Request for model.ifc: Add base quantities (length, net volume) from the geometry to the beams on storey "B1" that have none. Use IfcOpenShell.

First a look at what the model holds.

```python
import ifcopenshell
import ifcopenshell.util.element
import ifcopenshell.util.unit

model = ifcopenshell.open("model.ifc")
print(model.schema)
for unit_type in ("LENGTHUNIT", "AREAUNIT", "VOLUMEUNIT"):
    print(unit_type, ifcopenshell.util.unit.calculate_unit_scale(model, unit_type))
storey = next(s for s in model.by_type("IfcBuildingStorey") if s.Name == "B1")
beams = [e for e in ifcopenshell.util.element.get_decomposition(storey) if e.is_a("IfcBeam")]
for e in sorted(beams, key=lambda e: e.id()):
    print(e.id(), e.is_a(), e.Name, list(ifcopenshell.util.element.get_psets(e, qtos_only=True)), sep=" | ")
```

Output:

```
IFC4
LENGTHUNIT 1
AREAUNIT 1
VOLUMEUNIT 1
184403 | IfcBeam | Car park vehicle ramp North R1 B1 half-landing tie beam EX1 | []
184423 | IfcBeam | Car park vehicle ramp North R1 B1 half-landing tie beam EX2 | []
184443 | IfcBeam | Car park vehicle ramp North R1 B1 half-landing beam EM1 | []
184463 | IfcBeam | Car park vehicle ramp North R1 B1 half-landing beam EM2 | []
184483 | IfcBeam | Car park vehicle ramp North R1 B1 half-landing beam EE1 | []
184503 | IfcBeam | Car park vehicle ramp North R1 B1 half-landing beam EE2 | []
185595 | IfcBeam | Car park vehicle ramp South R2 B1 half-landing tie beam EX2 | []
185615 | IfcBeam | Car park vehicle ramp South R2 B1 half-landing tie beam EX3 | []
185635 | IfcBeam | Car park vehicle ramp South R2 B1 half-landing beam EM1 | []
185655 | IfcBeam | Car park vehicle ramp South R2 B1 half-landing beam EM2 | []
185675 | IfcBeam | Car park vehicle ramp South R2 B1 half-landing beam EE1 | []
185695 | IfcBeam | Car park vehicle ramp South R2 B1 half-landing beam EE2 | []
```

```python
import ifcopenshell
import ifcopenshell.api.pset
import ifcopenshell.geom
import ifcopenshell.util.element
import ifcopenshell.util.shape
import ifcopenshell.util.unit

model = ifcopenshell.open("model.ifc")
unit_scale = ifcopenshell.util.unit.calculate_unit_scale(model)
volume_scale = ifcopenshell.util.unit.calculate_unit_scale(model, "VOLUMEUNIT")
settings = ifcopenshell.geom.settings()

storey = next(s for s in model.by_type("IfcBuildingStorey") if s.Name == "B1")
beams = [e for e in ifcopenshell.util.element.get_decomposition(storey) if e.is_a("IfcBeam")]

for e in sorted(beams, key=lambda e: e.id()):
    if ifcopenshell.util.element.get_psets(e, qtos_only=True, should_inherit=False):
        continue
    # Geometry comes back in metres, in the element's own axes.
    shape = ifcopenshell.geom.create_shape(settings, e)
    values = {
        "Length": ifcopenshell.util.shape.get_max_xyz(shape.geometry) / unit_scale,
        "NetVolume": ifcopenshell.util.shape.get_volume(shape.geometry) / volume_scale,
    }
    qto = ifcopenshell.api.pset.add_qto(model, product=e, name="Qto_BeamBaseQuantities")
    ifcopenshell.api.pset.edit_qto(model, qto=qto, properties=values)
    print(e.id(), {k: round(v, 3) for k, v in values.items()})

model.write("model-out.ifc")
```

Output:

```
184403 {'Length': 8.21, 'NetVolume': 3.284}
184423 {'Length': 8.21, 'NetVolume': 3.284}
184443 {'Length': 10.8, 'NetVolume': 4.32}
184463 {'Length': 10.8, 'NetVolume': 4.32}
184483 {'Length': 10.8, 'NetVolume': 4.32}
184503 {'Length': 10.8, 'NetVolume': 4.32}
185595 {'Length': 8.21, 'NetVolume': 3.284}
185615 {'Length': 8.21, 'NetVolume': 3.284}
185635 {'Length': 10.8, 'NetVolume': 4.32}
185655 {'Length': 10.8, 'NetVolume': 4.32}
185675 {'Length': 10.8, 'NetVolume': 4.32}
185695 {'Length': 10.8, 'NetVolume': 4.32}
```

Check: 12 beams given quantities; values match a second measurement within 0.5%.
